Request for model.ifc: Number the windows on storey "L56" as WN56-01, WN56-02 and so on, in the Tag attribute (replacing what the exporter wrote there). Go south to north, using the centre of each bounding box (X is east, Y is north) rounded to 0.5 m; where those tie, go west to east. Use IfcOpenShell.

First a look at what the model holds.

```python
import ifcopenshell
import ifcopenshell.util.element
import ifcopenshell.util.placement

model = ifcopenshell.open("model.ifc")
print(model.schema)
storey = next(s for s in model.by_type("IfcBuildingStorey") if s.Name == "L56")
windows = [e for e in ifcopenshell.util.element.get_decomposition(storey) if e.is_a("IfcWindow")]
for e in sorted(windows, key=lambda e: e.id()):
    origin = ifcopenshell.util.placement.get_local_placement(e.ObjectPlacement)[:3, 3]
    print(e.id(), e.Tag, e.Name, origin.round(2) + 0.0, sep=" | ")
```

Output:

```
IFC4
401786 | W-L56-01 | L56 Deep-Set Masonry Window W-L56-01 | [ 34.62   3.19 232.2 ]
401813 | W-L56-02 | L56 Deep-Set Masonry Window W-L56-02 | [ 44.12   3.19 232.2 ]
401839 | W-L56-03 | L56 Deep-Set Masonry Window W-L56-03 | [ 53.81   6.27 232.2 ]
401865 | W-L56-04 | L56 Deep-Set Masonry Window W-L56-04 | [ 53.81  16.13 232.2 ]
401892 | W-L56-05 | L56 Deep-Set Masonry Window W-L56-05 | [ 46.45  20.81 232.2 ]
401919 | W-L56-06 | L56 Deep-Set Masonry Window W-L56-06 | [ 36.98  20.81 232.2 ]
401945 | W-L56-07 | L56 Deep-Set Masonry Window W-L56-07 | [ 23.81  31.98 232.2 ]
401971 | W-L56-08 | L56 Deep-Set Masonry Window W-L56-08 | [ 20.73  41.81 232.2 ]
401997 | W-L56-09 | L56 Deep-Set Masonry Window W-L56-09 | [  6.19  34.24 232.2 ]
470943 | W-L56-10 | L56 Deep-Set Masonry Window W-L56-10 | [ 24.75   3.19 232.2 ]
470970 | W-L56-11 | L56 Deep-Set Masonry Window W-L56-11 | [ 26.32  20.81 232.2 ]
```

```python
import ifcopenshell
import ifcopenshell.geom
import ifcopenshell.util.element
import ifcopenshell.util.shape

model = ifcopenshell.open("model.ifc")
settings = ifcopenshell.geom.settings()
settings.set("use-world-coords", True)


def centre(element):
    shape = ifcopenshell.geom.create_shape(settings, element)
    return ifcopenshell.util.shape.get_bbox_centroid(shape.geometry)


storey = next(s for s in model.by_type("IfcBuildingStorey") if s.Name == "L56")
windows = [e for e in ifcopenshell.util.element.get_decomposition(storey) if e.is_a("IfcWindow")]

# Insertion points can sit at a corner or the storey origin, so sort by the geometry (in metres).
centres = {e: centre(e) for e in windows}
windows.sort(key=lambda e: (round(centres[e][1] / 0.5), centres[e][0]))

for i, e in enumerate(windows, start=1):
    number = f"WN56-{i:02d}"
    e.Tag = number
    print(e.id(), number)

model.write("model_v2.ifc")
```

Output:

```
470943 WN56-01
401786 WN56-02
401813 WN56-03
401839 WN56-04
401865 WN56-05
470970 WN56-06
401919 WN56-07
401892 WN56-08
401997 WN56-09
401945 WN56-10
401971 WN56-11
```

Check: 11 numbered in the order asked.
